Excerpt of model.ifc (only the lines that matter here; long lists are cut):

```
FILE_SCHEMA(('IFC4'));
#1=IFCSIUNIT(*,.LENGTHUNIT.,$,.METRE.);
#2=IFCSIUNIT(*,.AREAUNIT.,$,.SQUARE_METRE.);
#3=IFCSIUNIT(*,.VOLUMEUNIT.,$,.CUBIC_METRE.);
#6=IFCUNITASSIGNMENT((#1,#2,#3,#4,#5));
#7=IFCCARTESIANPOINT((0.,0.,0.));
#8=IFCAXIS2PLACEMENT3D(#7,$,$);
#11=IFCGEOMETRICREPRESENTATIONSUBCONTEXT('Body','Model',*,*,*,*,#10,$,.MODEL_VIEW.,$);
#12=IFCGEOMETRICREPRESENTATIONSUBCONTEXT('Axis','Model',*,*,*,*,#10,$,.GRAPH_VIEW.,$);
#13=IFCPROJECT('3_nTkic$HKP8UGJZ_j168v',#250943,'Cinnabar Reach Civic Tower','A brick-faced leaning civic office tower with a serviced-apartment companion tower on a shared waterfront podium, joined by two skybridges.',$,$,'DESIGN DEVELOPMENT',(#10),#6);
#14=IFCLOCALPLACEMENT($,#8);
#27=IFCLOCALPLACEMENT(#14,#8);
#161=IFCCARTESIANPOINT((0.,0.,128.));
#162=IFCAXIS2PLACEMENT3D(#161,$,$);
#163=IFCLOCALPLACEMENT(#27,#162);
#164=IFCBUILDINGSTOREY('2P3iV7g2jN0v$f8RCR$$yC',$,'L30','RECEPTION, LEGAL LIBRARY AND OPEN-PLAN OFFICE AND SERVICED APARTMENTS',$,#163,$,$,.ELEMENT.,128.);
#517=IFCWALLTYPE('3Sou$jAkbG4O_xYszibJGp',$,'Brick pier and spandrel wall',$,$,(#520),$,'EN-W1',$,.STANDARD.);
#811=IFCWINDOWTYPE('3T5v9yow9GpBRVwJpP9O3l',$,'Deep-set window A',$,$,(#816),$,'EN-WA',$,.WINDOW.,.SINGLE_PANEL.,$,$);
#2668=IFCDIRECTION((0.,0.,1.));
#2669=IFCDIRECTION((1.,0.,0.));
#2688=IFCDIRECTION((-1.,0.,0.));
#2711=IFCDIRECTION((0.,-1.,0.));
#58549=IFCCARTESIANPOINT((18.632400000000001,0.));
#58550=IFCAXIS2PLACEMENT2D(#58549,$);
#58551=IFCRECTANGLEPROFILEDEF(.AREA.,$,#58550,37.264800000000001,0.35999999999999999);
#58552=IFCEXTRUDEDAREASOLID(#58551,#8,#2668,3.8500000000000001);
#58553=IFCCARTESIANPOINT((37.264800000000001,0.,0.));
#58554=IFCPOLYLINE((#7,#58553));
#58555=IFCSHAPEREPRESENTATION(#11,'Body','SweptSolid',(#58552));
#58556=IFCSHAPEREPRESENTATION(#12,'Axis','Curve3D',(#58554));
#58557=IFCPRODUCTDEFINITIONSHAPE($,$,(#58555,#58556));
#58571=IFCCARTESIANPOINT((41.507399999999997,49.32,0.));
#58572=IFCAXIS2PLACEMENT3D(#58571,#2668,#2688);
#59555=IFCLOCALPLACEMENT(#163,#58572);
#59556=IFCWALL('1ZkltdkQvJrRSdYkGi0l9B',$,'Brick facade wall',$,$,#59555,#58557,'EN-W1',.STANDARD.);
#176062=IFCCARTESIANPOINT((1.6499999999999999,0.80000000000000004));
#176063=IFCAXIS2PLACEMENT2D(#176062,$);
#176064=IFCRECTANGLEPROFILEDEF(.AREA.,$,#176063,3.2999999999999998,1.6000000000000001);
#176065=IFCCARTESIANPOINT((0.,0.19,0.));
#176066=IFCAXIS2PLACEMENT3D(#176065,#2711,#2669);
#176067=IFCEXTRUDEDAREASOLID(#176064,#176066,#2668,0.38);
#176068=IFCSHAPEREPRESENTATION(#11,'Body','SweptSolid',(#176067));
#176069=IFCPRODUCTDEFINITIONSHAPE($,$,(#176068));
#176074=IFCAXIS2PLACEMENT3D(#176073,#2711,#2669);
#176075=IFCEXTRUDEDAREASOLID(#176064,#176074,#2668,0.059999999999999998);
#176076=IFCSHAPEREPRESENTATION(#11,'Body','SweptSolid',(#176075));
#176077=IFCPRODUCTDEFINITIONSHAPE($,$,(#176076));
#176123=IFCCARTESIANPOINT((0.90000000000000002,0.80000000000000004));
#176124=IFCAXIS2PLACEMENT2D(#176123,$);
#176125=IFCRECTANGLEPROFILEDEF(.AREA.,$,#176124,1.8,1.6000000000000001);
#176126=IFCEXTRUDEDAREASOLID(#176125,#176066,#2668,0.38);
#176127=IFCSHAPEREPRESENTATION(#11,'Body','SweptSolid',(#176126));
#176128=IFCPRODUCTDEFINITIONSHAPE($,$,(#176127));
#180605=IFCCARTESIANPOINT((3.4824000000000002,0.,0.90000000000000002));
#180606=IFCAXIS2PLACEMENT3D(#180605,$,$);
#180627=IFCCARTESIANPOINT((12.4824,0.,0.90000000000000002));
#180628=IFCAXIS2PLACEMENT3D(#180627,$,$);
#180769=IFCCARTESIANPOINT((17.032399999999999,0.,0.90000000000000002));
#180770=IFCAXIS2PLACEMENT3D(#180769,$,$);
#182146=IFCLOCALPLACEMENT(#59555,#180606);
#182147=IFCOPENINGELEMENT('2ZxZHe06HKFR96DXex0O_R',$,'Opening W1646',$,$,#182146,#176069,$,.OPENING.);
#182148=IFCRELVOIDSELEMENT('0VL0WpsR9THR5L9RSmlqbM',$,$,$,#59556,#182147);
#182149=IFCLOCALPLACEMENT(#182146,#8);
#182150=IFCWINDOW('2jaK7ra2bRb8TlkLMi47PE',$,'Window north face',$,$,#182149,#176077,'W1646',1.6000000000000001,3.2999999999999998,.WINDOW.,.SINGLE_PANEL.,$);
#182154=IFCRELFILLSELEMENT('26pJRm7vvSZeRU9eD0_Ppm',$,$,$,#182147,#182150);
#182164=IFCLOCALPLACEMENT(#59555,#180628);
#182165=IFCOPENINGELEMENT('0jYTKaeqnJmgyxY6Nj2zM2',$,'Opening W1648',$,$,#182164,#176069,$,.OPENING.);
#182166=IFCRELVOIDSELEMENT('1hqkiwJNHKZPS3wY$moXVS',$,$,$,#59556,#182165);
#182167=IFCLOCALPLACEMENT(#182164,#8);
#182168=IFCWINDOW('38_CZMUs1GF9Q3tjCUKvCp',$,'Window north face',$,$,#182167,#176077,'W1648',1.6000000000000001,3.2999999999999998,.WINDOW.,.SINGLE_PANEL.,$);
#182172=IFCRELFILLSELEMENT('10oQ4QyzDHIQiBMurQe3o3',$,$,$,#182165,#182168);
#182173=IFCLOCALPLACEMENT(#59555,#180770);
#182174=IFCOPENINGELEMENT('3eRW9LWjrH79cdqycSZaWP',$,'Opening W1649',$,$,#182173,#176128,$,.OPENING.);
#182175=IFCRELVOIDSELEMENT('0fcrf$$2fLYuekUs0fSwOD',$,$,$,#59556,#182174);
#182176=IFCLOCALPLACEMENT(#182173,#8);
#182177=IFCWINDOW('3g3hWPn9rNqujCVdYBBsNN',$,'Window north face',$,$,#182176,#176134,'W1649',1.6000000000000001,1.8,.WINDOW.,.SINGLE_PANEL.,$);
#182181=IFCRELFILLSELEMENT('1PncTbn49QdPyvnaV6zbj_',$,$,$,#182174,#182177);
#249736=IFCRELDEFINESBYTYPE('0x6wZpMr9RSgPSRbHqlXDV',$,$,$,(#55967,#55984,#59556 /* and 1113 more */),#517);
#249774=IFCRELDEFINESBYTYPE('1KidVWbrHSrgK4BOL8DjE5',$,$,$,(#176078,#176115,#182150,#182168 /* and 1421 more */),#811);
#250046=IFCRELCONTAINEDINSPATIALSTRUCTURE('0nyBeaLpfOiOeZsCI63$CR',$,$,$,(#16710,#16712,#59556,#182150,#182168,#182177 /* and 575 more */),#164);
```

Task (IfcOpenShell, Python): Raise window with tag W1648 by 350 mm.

```python
import numpy as np
import ifcopenshell
import ifcopenshell.api.geometry
import ifcopenshell.util.placement
import ifcopenshell.util.unit

model = ifcopenshell.open("model.ifc")
unit_scale = ifcopenshell.util.unit.calculate_unit_scale(model)

window = model.by_guid("38_CZMUs1GF9Q3tjCUKvCp")
opening = window.FillsVoids[0].RelatingOpeningElement
dz = 0.35 / unit_scale

shift = np.array([0.0, 0.0, dz])
# The window is placed relative to its opening, so it follows when the opening moves.
matrix = ifcopenshell.util.placement.get_local_placement(opening.ObjectPlacement)
matrix[:3, 3] += shift
ifcopenshell.api.geometry.edit_object_placement(
    model, product=opening, matrix=matrix, is_si=False, should_transform_children=True
)

print(f"moved by {dz * unit_scale:+.3f} m")

model.write("model_rev.ifc")
```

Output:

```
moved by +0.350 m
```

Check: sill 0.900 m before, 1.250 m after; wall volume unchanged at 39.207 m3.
